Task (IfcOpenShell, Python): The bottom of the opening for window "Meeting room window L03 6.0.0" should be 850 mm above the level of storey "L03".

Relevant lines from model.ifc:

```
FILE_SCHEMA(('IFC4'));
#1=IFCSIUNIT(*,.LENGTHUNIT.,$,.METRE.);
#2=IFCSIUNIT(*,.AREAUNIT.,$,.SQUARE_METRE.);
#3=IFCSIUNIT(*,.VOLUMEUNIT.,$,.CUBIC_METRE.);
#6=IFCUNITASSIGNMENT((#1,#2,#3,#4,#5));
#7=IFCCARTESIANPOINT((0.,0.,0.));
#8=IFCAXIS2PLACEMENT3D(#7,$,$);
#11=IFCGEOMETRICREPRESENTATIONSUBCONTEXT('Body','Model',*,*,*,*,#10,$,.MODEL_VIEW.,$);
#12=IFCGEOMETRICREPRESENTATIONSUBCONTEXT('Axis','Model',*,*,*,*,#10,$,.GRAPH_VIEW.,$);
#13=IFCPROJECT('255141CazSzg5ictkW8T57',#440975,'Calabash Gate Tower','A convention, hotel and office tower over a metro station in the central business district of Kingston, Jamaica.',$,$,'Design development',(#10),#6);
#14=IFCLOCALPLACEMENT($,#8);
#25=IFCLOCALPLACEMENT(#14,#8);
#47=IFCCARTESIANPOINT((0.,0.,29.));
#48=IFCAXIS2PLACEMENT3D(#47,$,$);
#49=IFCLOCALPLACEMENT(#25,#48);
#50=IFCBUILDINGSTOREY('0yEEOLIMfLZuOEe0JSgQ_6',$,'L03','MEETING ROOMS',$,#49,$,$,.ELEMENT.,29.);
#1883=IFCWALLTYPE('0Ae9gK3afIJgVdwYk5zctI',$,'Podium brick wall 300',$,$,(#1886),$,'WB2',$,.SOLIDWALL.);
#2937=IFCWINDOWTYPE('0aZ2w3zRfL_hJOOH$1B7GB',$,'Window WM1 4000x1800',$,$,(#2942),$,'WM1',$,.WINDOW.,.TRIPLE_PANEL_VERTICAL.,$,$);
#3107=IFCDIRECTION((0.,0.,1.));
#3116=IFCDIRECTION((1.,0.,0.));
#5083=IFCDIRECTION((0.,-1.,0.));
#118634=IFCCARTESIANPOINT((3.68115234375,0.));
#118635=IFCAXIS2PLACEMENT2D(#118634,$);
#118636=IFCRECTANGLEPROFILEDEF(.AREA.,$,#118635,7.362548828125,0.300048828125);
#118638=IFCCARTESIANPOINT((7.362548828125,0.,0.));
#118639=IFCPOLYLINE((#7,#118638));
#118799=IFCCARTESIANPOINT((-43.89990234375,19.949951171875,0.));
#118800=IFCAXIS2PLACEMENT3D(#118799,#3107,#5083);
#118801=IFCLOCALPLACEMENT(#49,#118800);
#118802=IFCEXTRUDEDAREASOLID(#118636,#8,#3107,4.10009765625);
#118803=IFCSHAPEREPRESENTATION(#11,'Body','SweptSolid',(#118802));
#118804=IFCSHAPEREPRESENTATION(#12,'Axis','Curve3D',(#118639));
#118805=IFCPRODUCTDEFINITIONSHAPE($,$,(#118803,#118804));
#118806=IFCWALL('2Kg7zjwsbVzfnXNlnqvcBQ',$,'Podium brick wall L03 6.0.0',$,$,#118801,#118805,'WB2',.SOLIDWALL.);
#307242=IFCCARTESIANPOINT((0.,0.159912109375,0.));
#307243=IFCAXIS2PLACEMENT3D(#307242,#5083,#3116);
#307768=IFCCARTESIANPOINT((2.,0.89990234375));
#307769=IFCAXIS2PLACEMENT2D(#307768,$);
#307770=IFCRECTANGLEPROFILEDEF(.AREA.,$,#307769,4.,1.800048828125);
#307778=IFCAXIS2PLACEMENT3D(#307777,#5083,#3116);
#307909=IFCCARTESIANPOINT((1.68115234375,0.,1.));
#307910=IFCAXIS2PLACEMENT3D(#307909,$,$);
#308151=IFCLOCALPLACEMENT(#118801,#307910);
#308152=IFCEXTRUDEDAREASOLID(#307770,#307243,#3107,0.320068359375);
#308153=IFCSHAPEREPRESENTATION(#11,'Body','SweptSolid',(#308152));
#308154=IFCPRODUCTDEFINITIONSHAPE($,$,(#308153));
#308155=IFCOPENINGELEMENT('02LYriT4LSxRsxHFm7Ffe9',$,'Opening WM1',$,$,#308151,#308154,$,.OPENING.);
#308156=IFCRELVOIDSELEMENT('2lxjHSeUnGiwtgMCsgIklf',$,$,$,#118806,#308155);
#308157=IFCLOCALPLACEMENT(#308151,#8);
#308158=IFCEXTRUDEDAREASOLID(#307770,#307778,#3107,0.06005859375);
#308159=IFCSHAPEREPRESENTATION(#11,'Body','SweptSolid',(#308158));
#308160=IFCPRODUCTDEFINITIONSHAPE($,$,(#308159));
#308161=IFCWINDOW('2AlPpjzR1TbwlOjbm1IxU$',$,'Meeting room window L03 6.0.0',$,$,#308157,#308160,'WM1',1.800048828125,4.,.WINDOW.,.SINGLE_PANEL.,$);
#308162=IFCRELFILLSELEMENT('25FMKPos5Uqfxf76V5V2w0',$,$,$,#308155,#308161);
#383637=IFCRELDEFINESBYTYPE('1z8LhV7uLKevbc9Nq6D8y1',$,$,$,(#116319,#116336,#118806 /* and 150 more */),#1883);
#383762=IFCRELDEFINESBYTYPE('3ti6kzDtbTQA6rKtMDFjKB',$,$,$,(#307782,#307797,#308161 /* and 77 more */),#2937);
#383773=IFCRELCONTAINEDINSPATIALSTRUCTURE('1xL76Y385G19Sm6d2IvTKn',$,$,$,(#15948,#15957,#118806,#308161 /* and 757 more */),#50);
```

```python
import numpy as np
import ifcopenshell
import ifcopenshell.api.geometry
import ifcopenshell.geom
import ifcopenshell.util.element
import ifcopenshell.util.placement
import ifcopenshell.util.shape
import ifcopenshell.util.unit

model = ifcopenshell.open("model.ifc")
unit_scale = ifcopenshell.util.unit.calculate_unit_scale(model)

window = model.by_guid("2AlPpjzR1TbwlOjbm1IxU$")
opening = window.FillsVoids[0].RelatingOpeningElement
storey = ifcopenshell.util.element.get_container(window, ifc_class="IfcBuildingStorey")
level = ifcopenshell.util.placement.get_local_placement(storey.ObjectPlacement)[2, 3]

# The opening's origin need not be at the sill, so measure its lowest point.
shape = ifcopenshell.geom.create_shape(ifcopenshell.geom.settings(), opening)
bottom = ifcopenshell.util.shape.get_shape_bottom_elevation(shape, shape.geometry) / unit_scale
dz = level + 0.85 - bottom

shift = np.array([0.0, 0.0, dz])
# The window is placed relative to its opening, so it follows when the opening moves.
matrix = ifcopenshell.util.placement.get_local_placement(opening.ObjectPlacement)
matrix[:3, 3] += shift
ifcopenshell.api.geometry.edit_object_placement(
    model, product=opening, matrix=matrix, is_si=False, should_transform_children=True
)

print(f"moved by {dz * unit_scale:+.3f} m")

model.write("model_edited.ifc")
```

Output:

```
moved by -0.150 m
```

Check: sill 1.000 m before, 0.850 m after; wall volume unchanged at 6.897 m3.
